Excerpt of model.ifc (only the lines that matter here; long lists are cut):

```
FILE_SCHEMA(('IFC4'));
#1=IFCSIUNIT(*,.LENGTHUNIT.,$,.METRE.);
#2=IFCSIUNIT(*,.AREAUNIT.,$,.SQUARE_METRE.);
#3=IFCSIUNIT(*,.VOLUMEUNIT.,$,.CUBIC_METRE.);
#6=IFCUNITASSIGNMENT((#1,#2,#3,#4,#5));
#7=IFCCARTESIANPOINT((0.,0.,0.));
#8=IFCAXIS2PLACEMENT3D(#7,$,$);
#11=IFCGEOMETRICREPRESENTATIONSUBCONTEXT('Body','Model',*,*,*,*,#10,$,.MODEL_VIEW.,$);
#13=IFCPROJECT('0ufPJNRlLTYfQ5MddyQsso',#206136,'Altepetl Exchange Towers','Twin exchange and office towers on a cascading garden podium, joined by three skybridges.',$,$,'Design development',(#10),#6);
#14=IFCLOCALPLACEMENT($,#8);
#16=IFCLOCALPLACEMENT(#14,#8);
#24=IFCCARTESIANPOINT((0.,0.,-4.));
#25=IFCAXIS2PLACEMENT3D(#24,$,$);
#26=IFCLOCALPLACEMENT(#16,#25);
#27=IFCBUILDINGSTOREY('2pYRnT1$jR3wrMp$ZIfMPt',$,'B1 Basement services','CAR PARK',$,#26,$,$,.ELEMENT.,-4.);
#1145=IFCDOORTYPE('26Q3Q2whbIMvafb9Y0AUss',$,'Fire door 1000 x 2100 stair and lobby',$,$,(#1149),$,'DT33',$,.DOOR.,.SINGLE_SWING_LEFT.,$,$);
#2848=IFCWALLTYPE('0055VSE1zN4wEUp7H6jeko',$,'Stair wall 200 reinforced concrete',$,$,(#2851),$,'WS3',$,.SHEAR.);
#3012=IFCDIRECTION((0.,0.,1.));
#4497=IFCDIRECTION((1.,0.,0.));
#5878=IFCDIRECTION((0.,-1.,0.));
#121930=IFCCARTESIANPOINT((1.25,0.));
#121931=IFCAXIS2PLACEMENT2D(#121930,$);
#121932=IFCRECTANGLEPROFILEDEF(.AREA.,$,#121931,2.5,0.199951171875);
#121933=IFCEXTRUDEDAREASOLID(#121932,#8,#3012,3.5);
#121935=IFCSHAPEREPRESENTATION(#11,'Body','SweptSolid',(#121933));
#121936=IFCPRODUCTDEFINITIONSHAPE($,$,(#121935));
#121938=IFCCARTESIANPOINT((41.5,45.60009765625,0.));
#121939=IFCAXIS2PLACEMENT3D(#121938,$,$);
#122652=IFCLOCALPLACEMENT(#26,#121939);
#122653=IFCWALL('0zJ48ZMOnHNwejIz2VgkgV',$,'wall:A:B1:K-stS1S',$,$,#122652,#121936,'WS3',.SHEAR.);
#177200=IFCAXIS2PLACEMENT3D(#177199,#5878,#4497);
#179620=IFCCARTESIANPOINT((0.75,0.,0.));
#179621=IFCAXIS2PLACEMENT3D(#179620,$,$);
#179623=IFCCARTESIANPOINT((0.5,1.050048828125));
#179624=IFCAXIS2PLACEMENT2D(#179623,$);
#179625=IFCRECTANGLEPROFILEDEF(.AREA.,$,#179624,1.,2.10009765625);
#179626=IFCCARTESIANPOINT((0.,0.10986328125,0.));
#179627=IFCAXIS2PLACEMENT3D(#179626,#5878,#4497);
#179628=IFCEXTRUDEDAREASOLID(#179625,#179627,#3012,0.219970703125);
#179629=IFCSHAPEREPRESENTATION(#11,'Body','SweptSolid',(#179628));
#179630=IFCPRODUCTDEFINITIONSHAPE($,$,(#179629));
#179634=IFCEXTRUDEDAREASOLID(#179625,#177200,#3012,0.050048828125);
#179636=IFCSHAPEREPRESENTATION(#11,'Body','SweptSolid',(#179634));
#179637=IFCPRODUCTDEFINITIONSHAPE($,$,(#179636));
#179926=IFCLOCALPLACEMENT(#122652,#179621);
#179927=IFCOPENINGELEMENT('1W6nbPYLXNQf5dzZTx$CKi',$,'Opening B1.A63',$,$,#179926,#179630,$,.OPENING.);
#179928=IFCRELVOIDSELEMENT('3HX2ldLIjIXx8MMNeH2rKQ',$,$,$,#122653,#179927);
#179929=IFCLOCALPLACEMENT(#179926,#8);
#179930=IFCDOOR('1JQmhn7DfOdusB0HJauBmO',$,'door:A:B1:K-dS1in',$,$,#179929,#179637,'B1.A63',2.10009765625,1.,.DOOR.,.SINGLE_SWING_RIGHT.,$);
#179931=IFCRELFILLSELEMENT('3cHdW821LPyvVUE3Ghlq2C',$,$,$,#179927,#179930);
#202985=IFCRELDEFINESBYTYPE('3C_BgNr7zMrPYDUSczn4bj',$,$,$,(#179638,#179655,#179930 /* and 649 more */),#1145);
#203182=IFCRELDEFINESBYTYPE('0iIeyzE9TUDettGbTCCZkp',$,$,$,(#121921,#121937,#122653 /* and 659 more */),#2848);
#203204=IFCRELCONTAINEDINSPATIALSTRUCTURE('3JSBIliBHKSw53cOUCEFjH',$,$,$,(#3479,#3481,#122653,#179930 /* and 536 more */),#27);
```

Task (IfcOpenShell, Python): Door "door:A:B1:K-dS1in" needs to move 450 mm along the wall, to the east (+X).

```python
import ifcopenshell
import ifcopenshell.api.geometry
import ifcopenshell.util.placement
import ifcopenshell.util.unit

model = ifcopenshell.open("model.ifc")
unit_scale = ifcopenshell.util.unit.calculate_unit_scale(model)

door = model.by_guid("1JQmhn7DfOdusB0HJauBmO")
opening = door.FillsVoids[0].RelatingOpeningElement
wall = opening.VoidsElements[0].RelatingBuildingElement

wall_matrix = ifcopenshell.util.placement.get_local_placement(wall.ObjectPlacement)
shift = wall_matrix[:3, 0] * 0.45 / unit_scale
before = ifcopenshell.util.placement.get_local_placement(door.ObjectPlacement)[:3, 3].copy()

# The door is placed relative to its opening, so it follows when the opening moves.
matrix = ifcopenshell.util.placement.get_local_placement(opening.ObjectPlacement)
matrix[:3, 3] += shift
ifcopenshell.api.geometry.edit_object_placement(
    model, product=opening, matrix=matrix, is_si=False, should_transform_children=True
)

after = ifcopenshell.util.placement.get_local_placement(door.ObjectPlacement)[:3, 3]
print("door moved by", (after - before).round(3) + 0.0)

model.write("model_edited.ifc")
```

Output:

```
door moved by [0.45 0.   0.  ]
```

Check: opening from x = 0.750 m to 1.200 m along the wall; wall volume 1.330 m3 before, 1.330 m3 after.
